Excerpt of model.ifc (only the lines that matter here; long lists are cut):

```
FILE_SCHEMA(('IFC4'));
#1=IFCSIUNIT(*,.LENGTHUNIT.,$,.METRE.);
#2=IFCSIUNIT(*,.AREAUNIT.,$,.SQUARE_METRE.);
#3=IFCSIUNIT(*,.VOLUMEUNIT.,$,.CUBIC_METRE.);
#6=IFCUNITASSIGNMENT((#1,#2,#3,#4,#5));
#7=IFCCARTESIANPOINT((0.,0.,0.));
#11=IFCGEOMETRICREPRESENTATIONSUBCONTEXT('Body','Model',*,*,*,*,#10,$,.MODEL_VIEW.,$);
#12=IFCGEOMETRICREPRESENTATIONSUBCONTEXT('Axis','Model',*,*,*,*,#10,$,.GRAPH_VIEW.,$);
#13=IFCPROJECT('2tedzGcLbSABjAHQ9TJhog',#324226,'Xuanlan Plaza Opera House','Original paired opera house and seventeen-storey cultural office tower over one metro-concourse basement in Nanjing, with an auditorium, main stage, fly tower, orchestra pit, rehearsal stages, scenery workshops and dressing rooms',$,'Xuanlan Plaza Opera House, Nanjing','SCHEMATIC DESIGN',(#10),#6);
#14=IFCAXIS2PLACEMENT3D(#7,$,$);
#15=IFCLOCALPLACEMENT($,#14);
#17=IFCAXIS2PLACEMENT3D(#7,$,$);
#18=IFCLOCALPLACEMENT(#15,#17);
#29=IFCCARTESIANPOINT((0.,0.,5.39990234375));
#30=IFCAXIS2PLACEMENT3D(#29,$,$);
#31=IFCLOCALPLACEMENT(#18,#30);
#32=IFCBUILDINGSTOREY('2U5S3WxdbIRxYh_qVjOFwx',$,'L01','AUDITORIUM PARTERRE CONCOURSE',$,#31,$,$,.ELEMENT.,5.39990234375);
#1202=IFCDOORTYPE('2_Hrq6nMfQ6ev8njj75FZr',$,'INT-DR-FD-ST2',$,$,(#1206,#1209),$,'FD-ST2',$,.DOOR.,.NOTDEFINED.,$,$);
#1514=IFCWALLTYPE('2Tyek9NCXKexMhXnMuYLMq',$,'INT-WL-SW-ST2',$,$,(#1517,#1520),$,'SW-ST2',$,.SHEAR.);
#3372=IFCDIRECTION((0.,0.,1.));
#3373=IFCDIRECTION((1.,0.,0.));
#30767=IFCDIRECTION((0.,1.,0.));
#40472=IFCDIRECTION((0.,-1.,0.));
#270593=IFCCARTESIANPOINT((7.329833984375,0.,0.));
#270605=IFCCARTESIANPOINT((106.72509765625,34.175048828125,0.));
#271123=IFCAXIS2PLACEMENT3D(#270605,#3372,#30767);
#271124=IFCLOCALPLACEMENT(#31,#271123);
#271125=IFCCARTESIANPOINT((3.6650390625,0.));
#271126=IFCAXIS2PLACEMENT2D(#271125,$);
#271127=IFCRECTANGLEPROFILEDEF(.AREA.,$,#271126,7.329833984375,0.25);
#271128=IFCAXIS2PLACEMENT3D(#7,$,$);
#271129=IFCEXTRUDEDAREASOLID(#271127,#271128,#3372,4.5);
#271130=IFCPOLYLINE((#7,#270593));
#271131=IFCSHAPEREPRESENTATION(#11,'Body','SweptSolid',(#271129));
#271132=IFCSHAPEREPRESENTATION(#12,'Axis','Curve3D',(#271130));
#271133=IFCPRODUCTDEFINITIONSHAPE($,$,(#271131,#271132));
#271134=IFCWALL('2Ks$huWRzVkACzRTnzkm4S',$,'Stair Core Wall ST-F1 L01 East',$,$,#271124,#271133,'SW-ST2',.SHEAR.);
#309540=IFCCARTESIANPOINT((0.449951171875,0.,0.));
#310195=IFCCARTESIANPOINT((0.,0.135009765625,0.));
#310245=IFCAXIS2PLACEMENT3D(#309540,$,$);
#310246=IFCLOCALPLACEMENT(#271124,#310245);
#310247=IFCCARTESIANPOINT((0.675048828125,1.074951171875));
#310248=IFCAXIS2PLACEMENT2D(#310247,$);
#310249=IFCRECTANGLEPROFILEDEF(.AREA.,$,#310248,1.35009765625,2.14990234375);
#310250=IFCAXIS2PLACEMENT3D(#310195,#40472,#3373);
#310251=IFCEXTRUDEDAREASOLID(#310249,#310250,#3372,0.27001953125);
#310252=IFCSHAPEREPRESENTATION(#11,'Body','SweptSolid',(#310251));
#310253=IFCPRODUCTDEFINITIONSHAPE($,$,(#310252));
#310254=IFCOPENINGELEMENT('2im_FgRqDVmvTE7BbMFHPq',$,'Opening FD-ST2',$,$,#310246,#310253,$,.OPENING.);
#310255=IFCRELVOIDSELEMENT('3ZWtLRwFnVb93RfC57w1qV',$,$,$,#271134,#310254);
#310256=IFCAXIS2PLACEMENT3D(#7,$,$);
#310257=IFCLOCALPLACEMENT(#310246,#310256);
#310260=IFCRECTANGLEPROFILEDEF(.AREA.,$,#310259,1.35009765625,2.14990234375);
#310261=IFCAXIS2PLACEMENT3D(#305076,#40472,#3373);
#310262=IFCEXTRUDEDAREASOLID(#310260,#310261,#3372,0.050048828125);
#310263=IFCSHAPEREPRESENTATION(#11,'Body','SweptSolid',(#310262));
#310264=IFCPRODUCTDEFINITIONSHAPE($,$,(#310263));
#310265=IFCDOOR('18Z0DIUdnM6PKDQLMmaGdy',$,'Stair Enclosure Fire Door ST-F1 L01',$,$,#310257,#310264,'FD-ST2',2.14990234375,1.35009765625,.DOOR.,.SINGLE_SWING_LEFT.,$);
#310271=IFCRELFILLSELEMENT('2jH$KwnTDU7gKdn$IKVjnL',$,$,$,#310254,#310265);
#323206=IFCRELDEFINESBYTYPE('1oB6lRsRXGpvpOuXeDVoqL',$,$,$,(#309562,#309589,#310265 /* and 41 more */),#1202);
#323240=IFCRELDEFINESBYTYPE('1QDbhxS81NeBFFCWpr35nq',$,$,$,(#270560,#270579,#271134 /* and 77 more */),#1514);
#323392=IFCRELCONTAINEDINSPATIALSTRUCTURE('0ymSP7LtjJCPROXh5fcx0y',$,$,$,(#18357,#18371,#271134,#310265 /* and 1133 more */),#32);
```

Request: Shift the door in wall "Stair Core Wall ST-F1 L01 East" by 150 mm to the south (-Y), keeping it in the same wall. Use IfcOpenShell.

```python
import ifcopenshell
import ifcopenshell.api.geometry
import ifcopenshell.util.placement
import ifcopenshell.util.unit

model = ifcopenshell.open("model.ifc")
unit_scale = ifcopenshell.util.unit.calculate_unit_scale(model)

door = model.by_guid("18Z0DIUdnM6PKDQLMmaGdy")
opening = door.FillsVoids[0].RelatingOpeningElement
wall = opening.VoidsElements[0].RelatingBuildingElement

wall_matrix = ifcopenshell.util.placement.get_local_placement(wall.ObjectPlacement)
shift = wall_matrix[:3, 0] * -0.15 / unit_scale
before = ifcopenshell.util.placement.get_local_placement(door.ObjectPlacement)[:3, 3].copy()

# The door is placed relative to its opening, so it follows when the opening moves.
matrix = ifcopenshell.util.placement.get_local_placement(opening.ObjectPlacement)
matrix[:3, 3] += shift
ifcopenshell.api.geometry.edit_object_placement(
    model, product=opening, matrix=matrix, is_si=False, should_transform_children=True
)

after = ifcopenshell.util.placement.get_local_placement(door.ObjectPlacement)[:3, 3]
print("door moved by", (after - before).round(3) + 0.0)

model.write("model_v2.ifc")
```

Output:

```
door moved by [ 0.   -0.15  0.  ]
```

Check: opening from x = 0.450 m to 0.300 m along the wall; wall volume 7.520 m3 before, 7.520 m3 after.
